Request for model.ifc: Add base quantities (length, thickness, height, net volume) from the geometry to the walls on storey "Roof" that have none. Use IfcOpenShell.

First a look at what the model holds.

```python
import ifcopenshell
import ifcopenshell.util.element
import ifcopenshell.util.unit

model = ifcopenshell.open("model.ifc")
print(model.schema)
for unit_type in ("LENGTHUNIT", "AREAUNIT", "VOLUMEUNIT"):
    print(unit_type, ifcopenshell.util.unit.calculate_unit_scale(model, unit_type))
storey = next(s for s in model.by_type("IfcBuildingStorey") if s.Name == "Roof")
walls = [e for e in ifcopenshell.util.element.get_decomposition(storey) if e.is_a("IfcWall")]
for e in sorted(walls, key=lambda e: e.id()):
    print(e.id(), e.is_a(), e.Name, list(ifcopenshell.util.element.get_psets(e, qtos_only=True)), sep=" | ")
```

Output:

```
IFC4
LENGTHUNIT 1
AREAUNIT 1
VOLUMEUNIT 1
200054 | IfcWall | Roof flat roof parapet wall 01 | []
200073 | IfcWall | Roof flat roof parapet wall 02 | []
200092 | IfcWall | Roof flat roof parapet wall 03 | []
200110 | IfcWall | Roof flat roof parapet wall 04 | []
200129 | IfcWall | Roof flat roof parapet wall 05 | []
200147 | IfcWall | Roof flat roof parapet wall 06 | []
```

```python
import ifcopenshell
import ifcopenshell.api.pset
import ifcopenshell.geom
import ifcopenshell.util.element
import ifcopenshell.util.shape
import ifcopenshell.util.unit

model = ifcopenshell.open("model.ifc")
unit_scale = ifcopenshell.util.unit.calculate_unit_scale(model)
volume_scale = ifcopenshell.util.unit.calculate_unit_scale(model, "VOLUMEUNIT")
settings = ifcopenshell.geom.settings()

storey = next(s for s in model.by_type("IfcBuildingStorey") if s.Name == "Roof")
walls = [e for e in ifcopenshell.util.element.get_decomposition(storey) if e.is_a("IfcWall")]

for e in sorted(walls, key=lambda e: e.id()):
    if ifcopenshell.util.element.get_psets(e, qtos_only=True, should_inherit=False):
        continue
    # Geometry comes back in metres, in the element's own axes.
    shape = ifcopenshell.geom.create_shape(settings, e)
    values = {
        "Length": ifcopenshell.util.shape.get_x(shape.geometry) / unit_scale,
        "Width": ifcopenshell.util.shape.get_y(shape.geometry) / unit_scale,
        "Height": ifcopenshell.util.shape.get_z(shape.geometry) / unit_scale,
        "NetVolume": ifcopenshell.util.shape.get_volume(shape.geometry) / volume_scale,
    }
    qto = ifcopenshell.api.pset.add_qto(model, product=e, name="Qto_WallBaseQuantities")
    ifcopenshell.api.pset.edit_qto(model, qto=qto, properties=values)
    print(e.id(), {k: round(v, 3) for k, v in values.items()})

model.write("model-out.ifc")
```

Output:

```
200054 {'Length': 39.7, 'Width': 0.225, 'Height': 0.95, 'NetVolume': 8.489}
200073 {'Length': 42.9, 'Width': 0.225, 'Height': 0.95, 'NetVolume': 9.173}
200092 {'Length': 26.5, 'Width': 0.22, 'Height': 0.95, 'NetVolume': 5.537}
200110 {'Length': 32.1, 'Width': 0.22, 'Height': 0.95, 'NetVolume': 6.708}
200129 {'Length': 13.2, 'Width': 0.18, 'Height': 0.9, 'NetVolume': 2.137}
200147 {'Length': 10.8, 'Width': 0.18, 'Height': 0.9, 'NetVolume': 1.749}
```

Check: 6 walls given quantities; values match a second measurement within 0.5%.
